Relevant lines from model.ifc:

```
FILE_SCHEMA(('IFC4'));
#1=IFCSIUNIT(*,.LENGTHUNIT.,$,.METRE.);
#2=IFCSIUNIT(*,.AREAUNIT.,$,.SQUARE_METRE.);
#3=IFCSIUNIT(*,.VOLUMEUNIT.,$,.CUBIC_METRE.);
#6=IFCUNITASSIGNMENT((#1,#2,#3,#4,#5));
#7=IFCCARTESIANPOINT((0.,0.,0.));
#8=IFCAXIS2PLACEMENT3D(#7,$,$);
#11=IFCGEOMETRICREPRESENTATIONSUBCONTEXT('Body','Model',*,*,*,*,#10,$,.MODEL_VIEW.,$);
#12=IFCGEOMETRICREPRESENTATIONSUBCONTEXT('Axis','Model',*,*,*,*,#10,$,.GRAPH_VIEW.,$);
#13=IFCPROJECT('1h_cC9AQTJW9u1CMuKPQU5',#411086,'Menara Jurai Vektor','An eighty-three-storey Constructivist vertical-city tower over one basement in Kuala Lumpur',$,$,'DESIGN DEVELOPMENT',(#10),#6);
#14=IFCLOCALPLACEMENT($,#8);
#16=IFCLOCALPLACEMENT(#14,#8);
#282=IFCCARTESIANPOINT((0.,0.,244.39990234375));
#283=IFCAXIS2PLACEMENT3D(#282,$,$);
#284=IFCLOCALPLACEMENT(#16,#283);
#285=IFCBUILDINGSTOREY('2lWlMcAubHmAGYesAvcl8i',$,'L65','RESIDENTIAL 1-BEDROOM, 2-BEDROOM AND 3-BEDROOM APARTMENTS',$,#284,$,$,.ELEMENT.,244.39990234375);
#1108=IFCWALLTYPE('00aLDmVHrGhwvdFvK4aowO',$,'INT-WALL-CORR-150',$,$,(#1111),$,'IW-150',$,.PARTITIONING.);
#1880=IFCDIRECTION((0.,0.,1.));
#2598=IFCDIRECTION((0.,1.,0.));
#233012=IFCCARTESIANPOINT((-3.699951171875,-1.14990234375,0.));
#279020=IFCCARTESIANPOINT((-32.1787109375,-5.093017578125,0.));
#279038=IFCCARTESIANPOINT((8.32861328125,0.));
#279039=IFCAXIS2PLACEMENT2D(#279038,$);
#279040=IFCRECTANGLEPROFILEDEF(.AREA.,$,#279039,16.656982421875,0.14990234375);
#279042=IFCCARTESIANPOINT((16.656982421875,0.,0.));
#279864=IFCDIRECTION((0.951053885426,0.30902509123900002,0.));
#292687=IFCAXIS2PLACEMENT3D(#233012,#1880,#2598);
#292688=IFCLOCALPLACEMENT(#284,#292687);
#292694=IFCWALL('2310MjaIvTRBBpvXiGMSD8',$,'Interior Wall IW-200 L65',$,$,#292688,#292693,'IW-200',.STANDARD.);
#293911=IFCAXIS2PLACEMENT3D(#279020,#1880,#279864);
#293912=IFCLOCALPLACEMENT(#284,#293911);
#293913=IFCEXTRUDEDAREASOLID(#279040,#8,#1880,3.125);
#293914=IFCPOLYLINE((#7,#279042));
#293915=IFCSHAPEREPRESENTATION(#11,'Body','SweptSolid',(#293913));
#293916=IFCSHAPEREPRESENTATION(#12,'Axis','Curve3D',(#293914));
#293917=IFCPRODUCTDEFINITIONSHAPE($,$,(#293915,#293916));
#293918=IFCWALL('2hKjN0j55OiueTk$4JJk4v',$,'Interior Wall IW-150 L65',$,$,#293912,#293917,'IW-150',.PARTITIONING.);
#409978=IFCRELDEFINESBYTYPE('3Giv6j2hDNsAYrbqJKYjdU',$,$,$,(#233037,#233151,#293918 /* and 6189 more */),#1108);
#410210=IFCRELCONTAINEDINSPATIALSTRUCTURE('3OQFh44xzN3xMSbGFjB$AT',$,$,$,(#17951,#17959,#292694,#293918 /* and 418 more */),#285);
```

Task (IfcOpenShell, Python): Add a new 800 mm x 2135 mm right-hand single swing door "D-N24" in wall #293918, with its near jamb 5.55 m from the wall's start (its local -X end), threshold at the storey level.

```python
import numpy as np
import ifcopenshell
import ifcopenshell.api.feature
import ifcopenshell.api.geometry
import ifcopenshell.api.root
import ifcopenshell.api.spatial
import ifcopenshell.geom
import ifcopenshell.util.element
import ifcopenshell.util.placement
import ifcopenshell.util.representation
import ifcopenshell.util.shape
import ifcopenshell.util.unit

model = ifcopenshell.open("model.ifc")
unit_scale = ifcopenshell.util.unit.calculate_unit_scale(model)
settings = ifcopenshell.geom.settings()


def volume(element):
    """Net volume in cubic metres, openings subtracted."""
    shape = ifcopenshell.geom.create_shape(settings, element)
    return ifcopenshell.util.shape.get_volume(shape.geometry)


wall = model.by_id(293918)
storey = ifcopenshell.util.element.get_container(wall, ifc_class="IfcBuildingStorey")
context = ifcopenshell.util.representation.get_context(model, "Model", "Body", "MODEL_VIEW")
before = volume(wall)

width, height, from_end, sill = 0.8, 2.135, 5.55, 0.0  # metres

# The wall runs along its own X axis, and the end named is its -X end.
wall_shape = ifcopenshell.geom.create_shape(settings, wall)
x, y, z = ifcopenshell.util.shape.get_vertices(wall_shape.geometry).T
start = x.min() + from_end
face, thickness = float(y.min()), float(y.max() - y.min())
wall_matrix = ifcopenshell.util.placement.get_local_placement(wall.ObjectPlacement)
level = ifcopenshell.util.placement.get_local_placement(storey.ObjectPlacement)[2, 3]


def in_wall(x, y):
    """Placement at x, y metres in the wall's axes, at sill height."""
    matrix = wall_matrix.copy()
    matrix[:, 3] = wall_matrix @ np.array([x / unit_scale, y / unit_scale, 0.0, 1.0])
    matrix[2, 3] = level + sill / unit_scale
    return matrix


# Opening: a box that overshoots both wall faces by 50 mm.
opening = ifcopenshell.api.root.create_entity(model, ifc_class="IfcOpeningElement", predefined_type="OPENING")
box = ifcopenshell.api.geometry.add_wall_representation(
    model, context=context, length=width, height=height, thickness=thickness + 0.1
)
ifcopenshell.api.geometry.assign_representation(model, product=opening, representation=box)
ifcopenshell.api.geometry.edit_object_placement(model, product=opening, matrix=in_wall(start, face - 0.05), is_si=False)
ifcopenshell.api.feature.add_feature(model, feature=opening, element=wall)

door = ifcopenshell.api.root.create_entity(model, ifc_class="IfcDoor", name="D-N24", predefined_type="DOOR")
door.OverallWidth, door.OverallHeight = width / unit_scale, height / unit_scale
door.OperationType = "SINGLE_SWING_RIGHT"
body = ifcopenshell.api.geometry.add_door_representation(
    model,
    context=context,
    overall_width=door.OverallWidth,
    overall_height=door.OverallHeight,
    operation_type="SINGLE_SWING_RIGHT",
    lining_properties={"LiningDepth": thickness / unit_scale, "ThresholdDepth": thickness / unit_scale},
)
ifcopenshell.api.geometry.assign_representation(model, product=door, representation=body)
ifcopenshell.api.spatial.assign_container(model, products=[door], relating_structure=storey)
ifcopenshell.api.feature.add_filling(model, opening=opening, element=door)

# The lining spans the wall, so the door starts at the wall face.
ifcopenshell.api.geometry.edit_object_placement(model, product=door, matrix=in_wall(start, face), is_si=False)

after = volume(wall)

print(f"wall volume {before:.3f} -> {after:.3f} m3")

model.write("model-out.ifc")
```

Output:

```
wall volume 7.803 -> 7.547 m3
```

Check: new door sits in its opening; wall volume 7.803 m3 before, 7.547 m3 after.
